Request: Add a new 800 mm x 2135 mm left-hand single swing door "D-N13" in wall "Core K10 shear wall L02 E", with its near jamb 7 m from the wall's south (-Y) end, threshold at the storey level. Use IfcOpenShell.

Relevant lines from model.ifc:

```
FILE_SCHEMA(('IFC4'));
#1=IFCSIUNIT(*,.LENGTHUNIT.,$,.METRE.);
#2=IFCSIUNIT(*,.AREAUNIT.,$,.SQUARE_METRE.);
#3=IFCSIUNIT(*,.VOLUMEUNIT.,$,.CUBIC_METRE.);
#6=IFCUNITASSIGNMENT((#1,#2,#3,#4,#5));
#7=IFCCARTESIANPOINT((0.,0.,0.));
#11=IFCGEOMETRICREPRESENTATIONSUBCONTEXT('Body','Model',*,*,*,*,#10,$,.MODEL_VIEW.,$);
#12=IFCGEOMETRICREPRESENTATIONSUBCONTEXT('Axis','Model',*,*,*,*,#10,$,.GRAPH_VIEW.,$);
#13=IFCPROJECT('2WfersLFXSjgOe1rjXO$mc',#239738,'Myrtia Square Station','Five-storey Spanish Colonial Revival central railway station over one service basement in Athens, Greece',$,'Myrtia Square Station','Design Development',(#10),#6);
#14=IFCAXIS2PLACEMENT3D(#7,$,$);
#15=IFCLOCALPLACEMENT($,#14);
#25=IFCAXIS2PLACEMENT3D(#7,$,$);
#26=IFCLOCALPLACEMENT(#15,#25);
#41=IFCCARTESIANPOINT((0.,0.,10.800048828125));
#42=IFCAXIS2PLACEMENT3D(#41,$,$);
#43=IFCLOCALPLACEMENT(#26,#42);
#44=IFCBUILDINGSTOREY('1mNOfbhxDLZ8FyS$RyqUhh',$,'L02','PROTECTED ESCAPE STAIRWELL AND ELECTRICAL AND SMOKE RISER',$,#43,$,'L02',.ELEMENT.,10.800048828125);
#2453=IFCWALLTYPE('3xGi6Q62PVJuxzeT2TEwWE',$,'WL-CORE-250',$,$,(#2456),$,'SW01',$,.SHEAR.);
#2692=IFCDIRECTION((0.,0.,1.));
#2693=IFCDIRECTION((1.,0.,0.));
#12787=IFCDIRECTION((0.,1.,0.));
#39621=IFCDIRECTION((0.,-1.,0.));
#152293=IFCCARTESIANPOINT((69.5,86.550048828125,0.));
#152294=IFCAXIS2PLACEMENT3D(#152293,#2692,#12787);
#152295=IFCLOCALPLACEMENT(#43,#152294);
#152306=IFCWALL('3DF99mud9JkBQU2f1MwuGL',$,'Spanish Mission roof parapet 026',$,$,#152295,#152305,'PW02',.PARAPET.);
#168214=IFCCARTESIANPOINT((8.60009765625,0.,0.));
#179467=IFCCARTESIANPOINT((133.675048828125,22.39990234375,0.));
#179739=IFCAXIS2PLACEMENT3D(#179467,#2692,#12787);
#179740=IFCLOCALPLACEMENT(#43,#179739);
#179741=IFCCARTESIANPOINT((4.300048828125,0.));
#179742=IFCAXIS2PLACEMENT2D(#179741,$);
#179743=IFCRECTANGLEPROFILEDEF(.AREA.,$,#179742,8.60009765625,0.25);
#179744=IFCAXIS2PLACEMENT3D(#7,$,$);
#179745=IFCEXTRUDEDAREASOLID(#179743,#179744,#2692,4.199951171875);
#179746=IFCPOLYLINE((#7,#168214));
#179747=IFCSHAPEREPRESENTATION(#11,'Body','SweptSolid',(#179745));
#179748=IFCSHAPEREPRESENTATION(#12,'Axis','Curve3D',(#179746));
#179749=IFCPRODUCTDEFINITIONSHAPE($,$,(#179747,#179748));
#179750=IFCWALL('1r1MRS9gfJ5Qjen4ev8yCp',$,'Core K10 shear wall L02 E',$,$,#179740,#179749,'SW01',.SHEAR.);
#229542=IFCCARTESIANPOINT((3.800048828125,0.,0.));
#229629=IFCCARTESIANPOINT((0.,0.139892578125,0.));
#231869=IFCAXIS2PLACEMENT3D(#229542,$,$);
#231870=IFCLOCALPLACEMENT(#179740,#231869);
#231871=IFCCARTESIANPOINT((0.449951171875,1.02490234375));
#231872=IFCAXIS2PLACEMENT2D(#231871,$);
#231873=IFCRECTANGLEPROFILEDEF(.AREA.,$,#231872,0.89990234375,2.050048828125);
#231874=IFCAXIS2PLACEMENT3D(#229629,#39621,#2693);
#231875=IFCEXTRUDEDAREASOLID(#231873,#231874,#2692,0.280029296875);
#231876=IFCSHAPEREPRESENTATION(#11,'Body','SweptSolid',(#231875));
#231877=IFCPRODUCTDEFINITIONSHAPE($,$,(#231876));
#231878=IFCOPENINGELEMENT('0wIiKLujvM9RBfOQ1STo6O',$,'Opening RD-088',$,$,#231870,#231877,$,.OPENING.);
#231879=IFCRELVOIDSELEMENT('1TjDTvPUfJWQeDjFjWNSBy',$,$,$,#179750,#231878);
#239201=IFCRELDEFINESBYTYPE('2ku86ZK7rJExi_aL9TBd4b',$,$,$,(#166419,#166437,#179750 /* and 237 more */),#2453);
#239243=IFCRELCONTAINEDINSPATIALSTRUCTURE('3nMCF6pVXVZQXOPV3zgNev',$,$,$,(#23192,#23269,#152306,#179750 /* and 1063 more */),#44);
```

```python
import numpy as np
import ifcopenshell
import ifcopenshell.api.feature
import ifcopenshell.api.geometry
import ifcopenshell.api.root
import ifcopenshell.api.spatial
import ifcopenshell.geom
import ifcopenshell.util.element
import ifcopenshell.util.placement
import ifcopenshell.util.representation
import ifcopenshell.util.shape
import ifcopenshell.util.unit

model = ifcopenshell.open("model.ifc")
unit_scale = ifcopenshell.util.unit.calculate_unit_scale(model)
settings = ifcopenshell.geom.settings()


def volume(element):
    """Net volume in cubic metres, openings subtracted."""
    shape = ifcopenshell.geom.create_shape(settings, element)
    return ifcopenshell.util.shape.get_volume(shape.geometry)


wall = model.by_id(179750)
storey = ifcopenshell.util.element.get_container(wall, ifc_class="IfcBuildingStorey")
context = ifcopenshell.util.representation.get_context(model, "Model", "Body", "MODEL_VIEW")
before = volume(wall)

width, height, from_end, sill = 0.8, 2.135, 7, 0.0  # metres

# The wall runs along its own X axis, and the end named is its -X end.
wall_shape = ifcopenshell.geom.create_shape(settings, wall)
x, y, z = ifcopenshell.util.shape.get_vertices(wall_shape.geometry).T
start = x.min() + from_end
face, thickness = float(y.min()), float(y.max() - y.min())
wall_matrix = ifcopenshell.util.placement.get_local_placement(wall.ObjectPlacement)
level = ifcopenshell.util.placement.get_local_placement(storey.ObjectPlacement)[2, 3]


def in_wall(x, y):
    """Placement at x, y metres in the wall's axes, at sill height."""
    matrix = wall_matrix.copy()
    matrix[:, 3] = wall_matrix @ np.array([x / unit_scale, y / unit_scale, 0.0, 1.0])
    matrix[2, 3] = level + sill / unit_scale
    return matrix


# Opening: a box that overshoots both wall faces by 50 mm.
opening = ifcopenshell.api.root.create_entity(model, ifc_class="IfcOpeningElement", predefined_type="OPENING")
box = ifcopenshell.api.geometry.add_wall_representation(
    model, context=context, length=width, height=height, thickness=thickness + 0.1
)
ifcopenshell.api.geometry.assign_representation(model, product=opening, representation=box)
ifcopenshell.api.geometry.edit_object_placement(model, product=opening, matrix=in_wall(start, face - 0.05), is_si=False)
ifcopenshell.api.feature.add_feature(model, feature=opening, element=wall)

door = ifcopenshell.api.root.create_entity(model, ifc_class="IfcDoor", name="D-N13", predefined_type="DOOR")
door.OverallWidth, door.OverallHeight = width / unit_scale, height / unit_scale
door.OperationType = "SINGLE_SWING_LEFT"
body = ifcopenshell.api.geometry.add_door_representation(
    model,
    context=context,
    overall_width=door.OverallWidth,
    overall_height=door.OverallHeight,
    operation_type="SINGLE_SWING_LEFT",
    lining_properties={"LiningDepth": thickness / unit_scale, "ThresholdDepth": thickness / unit_scale},
)
ifcopenshell.api.geometry.assign_representation(model, product=door, representation=body)
ifcopenshell.api.spatial.assign_container(model, products=[door], relating_structure=storey)
ifcopenshell.api.feature.add_filling(model, opening=opening, element=door)

# The lining spans the wall, so the door starts at the wall face.
ifcopenshell.api.geometry.edit_object_placement(model, product=door, matrix=in_wall(start, face), is_si=False)

after = volume(wall)

print(f"wall volume {before:.3f} -> {after:.3f} m3")

model.write("model_v2.ifc")
```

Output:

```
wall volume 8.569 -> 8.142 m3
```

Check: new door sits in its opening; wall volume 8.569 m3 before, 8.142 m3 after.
